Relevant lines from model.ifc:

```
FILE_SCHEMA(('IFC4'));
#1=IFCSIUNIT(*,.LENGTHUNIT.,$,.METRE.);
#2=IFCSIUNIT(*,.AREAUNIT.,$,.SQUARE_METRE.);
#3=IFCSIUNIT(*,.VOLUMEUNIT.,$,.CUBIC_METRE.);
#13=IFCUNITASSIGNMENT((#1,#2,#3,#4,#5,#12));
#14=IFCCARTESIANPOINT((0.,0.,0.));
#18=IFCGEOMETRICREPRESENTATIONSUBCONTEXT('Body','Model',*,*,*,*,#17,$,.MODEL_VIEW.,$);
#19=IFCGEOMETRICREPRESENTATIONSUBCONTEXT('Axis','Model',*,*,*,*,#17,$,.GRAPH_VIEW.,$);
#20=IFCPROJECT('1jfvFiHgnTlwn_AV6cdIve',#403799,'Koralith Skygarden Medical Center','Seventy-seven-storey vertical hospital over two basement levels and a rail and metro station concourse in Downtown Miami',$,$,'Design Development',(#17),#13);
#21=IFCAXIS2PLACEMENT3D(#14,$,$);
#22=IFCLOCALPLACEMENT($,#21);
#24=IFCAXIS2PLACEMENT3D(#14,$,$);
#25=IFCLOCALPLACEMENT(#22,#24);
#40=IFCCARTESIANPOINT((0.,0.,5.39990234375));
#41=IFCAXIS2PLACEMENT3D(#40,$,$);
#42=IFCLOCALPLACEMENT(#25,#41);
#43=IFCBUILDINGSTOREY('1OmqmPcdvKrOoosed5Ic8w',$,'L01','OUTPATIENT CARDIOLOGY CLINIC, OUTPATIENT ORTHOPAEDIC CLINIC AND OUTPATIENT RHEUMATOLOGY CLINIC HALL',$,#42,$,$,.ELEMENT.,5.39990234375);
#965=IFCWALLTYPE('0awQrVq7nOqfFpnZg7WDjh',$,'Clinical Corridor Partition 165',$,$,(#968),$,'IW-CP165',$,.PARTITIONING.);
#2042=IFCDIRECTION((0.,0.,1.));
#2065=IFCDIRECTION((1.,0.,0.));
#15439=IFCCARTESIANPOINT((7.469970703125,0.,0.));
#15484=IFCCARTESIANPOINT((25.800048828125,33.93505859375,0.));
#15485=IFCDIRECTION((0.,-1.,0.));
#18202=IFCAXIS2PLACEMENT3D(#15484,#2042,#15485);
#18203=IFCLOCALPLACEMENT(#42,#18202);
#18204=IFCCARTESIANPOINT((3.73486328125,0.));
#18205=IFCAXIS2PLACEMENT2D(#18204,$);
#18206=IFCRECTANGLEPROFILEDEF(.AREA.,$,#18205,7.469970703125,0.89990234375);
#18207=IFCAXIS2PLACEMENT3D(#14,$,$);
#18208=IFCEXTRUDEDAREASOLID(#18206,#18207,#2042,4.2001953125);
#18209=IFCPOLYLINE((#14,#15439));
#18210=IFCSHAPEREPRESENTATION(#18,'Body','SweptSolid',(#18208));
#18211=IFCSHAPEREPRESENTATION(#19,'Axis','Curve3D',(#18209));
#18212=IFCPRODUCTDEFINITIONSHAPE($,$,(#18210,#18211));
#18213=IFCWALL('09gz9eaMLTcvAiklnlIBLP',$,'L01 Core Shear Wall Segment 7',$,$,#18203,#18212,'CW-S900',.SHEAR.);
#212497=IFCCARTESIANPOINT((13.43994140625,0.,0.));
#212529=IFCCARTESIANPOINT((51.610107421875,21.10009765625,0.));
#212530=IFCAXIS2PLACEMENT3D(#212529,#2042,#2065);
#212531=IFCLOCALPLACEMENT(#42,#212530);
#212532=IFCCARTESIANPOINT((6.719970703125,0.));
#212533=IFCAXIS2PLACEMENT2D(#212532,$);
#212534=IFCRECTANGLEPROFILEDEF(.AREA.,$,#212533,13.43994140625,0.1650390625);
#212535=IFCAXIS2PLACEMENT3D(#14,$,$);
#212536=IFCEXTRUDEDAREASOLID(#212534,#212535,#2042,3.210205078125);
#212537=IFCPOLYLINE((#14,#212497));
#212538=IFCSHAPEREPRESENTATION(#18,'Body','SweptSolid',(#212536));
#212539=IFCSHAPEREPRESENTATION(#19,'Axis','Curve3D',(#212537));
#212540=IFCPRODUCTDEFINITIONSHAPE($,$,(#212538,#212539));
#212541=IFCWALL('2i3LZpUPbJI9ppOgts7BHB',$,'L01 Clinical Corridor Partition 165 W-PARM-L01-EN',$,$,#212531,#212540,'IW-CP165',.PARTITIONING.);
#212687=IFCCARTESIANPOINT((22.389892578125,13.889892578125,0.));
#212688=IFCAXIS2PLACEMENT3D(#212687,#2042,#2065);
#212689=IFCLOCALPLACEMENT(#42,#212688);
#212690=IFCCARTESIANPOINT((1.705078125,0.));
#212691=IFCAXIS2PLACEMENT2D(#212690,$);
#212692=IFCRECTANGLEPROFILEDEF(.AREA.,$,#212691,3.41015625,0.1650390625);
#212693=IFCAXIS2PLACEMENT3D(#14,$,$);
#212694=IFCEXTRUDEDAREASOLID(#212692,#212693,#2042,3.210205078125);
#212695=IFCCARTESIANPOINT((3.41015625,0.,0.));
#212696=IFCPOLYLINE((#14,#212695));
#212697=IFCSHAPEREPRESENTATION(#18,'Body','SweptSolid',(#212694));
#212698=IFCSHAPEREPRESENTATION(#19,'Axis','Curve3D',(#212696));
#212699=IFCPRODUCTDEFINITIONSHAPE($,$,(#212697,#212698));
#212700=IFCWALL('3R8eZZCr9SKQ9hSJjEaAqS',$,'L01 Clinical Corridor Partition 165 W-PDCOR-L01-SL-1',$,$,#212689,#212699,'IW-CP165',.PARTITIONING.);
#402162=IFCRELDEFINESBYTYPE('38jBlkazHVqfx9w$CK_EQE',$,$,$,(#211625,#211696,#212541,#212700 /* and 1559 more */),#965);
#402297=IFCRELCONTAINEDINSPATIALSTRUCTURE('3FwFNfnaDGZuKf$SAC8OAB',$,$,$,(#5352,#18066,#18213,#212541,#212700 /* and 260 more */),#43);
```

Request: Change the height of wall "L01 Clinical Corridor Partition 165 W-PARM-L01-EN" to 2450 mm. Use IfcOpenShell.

```python
import ifcopenshell
import ifcopenshell.geom
import ifcopenshell.util.representation
import ifcopenshell.util.shape

model = ifcopenshell.open("model.ifc")
settings = ifcopenshell.geom.settings()


def volume(element):
    """Net volume in cubic metres, openings subtracted."""
    shape = ifcopenshell.geom.create_shape(settings, element)
    return ifcopenshell.util.shape.get_volume(shape.geometry)


wall = model.by_id(212541)
before = volume(wall)

body = ifcopenshell.util.representation.get_representation(wall, "Model", "Body")
solid = body.Items[0]
old_height = solid.Depth
solid.Depth = 2.45
after = volume(wall)

print(f"height {old_height:g} -> {solid.Depth:g}, volume {before:.3f} -> {after:.3f} m3")

model.write("model_v2.ifc")
```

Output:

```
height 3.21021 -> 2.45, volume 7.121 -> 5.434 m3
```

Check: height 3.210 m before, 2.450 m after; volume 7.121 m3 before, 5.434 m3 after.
